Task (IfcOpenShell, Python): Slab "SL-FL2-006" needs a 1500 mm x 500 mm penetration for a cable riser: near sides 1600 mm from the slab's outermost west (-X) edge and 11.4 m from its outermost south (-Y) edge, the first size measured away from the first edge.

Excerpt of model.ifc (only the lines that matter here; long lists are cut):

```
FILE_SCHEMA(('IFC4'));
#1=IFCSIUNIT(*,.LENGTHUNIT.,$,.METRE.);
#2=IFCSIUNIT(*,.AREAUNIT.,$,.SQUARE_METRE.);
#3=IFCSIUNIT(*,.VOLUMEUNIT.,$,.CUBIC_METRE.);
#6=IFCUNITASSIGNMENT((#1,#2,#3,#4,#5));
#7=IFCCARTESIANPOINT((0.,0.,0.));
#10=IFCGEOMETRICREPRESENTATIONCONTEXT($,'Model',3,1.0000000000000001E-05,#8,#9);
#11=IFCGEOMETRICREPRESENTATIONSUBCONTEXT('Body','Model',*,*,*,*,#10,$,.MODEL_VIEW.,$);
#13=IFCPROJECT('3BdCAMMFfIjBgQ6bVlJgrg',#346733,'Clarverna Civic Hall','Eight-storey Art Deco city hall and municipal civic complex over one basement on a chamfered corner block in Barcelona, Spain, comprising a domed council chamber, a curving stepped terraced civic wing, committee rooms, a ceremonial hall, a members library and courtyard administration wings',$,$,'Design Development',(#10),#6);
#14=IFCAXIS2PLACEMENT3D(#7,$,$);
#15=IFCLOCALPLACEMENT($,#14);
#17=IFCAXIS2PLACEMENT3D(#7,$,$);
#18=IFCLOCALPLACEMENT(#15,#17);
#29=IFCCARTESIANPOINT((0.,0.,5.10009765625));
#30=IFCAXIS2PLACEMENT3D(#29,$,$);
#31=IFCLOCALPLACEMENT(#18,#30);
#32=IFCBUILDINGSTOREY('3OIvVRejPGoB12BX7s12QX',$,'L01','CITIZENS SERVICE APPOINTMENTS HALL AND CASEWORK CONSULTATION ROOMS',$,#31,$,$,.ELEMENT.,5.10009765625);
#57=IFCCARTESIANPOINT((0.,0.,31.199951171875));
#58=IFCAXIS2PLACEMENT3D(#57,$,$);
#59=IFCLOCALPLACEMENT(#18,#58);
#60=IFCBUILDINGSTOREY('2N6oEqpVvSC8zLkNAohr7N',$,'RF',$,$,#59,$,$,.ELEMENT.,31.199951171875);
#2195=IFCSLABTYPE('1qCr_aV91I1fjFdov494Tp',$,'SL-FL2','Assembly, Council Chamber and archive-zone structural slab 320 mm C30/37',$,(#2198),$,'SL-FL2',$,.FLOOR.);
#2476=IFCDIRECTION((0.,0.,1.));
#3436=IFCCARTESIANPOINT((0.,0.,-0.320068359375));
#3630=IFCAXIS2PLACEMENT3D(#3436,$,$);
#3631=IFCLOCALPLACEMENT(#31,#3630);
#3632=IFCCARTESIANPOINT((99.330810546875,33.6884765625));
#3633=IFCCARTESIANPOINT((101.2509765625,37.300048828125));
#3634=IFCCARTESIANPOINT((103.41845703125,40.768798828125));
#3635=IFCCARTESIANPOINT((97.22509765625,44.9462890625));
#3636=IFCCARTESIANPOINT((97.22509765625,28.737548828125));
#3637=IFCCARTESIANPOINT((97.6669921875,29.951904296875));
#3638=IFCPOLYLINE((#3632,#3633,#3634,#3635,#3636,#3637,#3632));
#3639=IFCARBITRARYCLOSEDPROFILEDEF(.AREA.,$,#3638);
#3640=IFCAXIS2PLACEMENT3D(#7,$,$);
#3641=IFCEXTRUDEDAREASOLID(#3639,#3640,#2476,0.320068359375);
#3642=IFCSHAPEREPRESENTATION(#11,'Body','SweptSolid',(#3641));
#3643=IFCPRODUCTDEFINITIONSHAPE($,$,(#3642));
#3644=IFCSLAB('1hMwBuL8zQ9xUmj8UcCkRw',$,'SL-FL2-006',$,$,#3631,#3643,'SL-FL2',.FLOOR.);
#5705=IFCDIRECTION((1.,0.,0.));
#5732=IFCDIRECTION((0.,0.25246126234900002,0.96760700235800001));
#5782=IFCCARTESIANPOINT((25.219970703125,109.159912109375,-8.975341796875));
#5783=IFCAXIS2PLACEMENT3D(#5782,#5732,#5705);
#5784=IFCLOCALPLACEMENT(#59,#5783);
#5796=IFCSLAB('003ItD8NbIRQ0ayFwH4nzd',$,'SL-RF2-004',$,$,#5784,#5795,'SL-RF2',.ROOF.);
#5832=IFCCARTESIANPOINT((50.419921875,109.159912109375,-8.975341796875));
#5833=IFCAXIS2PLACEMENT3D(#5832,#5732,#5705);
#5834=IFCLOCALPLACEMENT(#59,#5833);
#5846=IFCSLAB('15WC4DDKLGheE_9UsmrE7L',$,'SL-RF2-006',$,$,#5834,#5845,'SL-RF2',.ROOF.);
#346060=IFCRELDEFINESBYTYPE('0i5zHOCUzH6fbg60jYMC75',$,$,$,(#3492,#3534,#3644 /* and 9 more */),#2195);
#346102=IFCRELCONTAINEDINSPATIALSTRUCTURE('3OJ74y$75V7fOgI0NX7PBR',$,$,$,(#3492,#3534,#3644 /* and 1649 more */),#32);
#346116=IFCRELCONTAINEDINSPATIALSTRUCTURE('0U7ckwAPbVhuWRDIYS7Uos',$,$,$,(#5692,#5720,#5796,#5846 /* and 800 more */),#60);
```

```python
import numpy as np
import ifcopenshell
import ifcopenshell.api.feature
import ifcopenshell.api.geometry
import ifcopenshell.api.root
import ifcopenshell.geom
import ifcopenshell.util.placement
import ifcopenshell.util.representation
import ifcopenshell.util.shape
import ifcopenshell.util.unit

model = ifcopenshell.open("model.ifc")
unit_scale = ifcopenshell.util.unit.calculate_unit_scale(model)
settings = ifcopenshell.geom.settings()


def volume(element):
    """Net volume in cubic metres, openings subtracted."""
    shape = ifcopenshell.geom.create_shape(settings, element)
    return ifcopenshell.util.shape.get_volume(shape.geometry)


slab = model.by_guid("1hMwBuL8zQ9xUmj8UcCkRw")
before = volume(slab)

# Extent in the slab's own axes, in metres. The edges named are its -X and -Y sides.
slab_shape = ifcopenshell.geom.create_shape(settings, slab)
vertices = ifcopenshell.util.shape.get_vertices(slab_shape.geometry)
x_min, y_min, bottom = vertices.min(axis=0)
top = vertices[:, 2].max()

opening = ifcopenshell.api.root.create_entity(model, ifc_class="IfcOpeningElement", name="Cable riser opening", predefined_type="OPENING")
context = ifcopenshell.util.representation.get_context(model, "Model", "Body", "MODEL_VIEW")
width, depth = 1.5, 0.5
outline = [(0.0, 0.0), (width, 0.0), (width, depth), (0.0, depth), (0.0, 0.0)]
# Overshoot both faces by 50 mm so the cut is clean.
shape = ifcopenshell.api.geometry.add_slab_representation(
    model, context=context, depth=top - bottom + 0.1, polyline=outline
)
ifcopenshell.api.geometry.assign_representation(model, product=opening, representation=shape)

matrix = ifcopenshell.util.placement.get_local_placement(slab.ObjectPlacement)
matrix[:, 3] = matrix @ np.append(np.array([x_min + 1.6, y_min + 11.4, bottom - 0.05]) / unit_scale, 1.0)
ifcopenshell.api.geometry.edit_object_placement(model, product=opening, matrix=matrix, is_si=False)
ifcopenshell.api.feature.add_feature(model, feature=opening, element=slab)

after = volume(slab)

print(f"slab volume {before:.3f} -> {after:.3f} m3")

model.write("model_rev.ifc")
```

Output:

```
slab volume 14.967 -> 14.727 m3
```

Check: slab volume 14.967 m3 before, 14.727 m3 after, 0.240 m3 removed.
